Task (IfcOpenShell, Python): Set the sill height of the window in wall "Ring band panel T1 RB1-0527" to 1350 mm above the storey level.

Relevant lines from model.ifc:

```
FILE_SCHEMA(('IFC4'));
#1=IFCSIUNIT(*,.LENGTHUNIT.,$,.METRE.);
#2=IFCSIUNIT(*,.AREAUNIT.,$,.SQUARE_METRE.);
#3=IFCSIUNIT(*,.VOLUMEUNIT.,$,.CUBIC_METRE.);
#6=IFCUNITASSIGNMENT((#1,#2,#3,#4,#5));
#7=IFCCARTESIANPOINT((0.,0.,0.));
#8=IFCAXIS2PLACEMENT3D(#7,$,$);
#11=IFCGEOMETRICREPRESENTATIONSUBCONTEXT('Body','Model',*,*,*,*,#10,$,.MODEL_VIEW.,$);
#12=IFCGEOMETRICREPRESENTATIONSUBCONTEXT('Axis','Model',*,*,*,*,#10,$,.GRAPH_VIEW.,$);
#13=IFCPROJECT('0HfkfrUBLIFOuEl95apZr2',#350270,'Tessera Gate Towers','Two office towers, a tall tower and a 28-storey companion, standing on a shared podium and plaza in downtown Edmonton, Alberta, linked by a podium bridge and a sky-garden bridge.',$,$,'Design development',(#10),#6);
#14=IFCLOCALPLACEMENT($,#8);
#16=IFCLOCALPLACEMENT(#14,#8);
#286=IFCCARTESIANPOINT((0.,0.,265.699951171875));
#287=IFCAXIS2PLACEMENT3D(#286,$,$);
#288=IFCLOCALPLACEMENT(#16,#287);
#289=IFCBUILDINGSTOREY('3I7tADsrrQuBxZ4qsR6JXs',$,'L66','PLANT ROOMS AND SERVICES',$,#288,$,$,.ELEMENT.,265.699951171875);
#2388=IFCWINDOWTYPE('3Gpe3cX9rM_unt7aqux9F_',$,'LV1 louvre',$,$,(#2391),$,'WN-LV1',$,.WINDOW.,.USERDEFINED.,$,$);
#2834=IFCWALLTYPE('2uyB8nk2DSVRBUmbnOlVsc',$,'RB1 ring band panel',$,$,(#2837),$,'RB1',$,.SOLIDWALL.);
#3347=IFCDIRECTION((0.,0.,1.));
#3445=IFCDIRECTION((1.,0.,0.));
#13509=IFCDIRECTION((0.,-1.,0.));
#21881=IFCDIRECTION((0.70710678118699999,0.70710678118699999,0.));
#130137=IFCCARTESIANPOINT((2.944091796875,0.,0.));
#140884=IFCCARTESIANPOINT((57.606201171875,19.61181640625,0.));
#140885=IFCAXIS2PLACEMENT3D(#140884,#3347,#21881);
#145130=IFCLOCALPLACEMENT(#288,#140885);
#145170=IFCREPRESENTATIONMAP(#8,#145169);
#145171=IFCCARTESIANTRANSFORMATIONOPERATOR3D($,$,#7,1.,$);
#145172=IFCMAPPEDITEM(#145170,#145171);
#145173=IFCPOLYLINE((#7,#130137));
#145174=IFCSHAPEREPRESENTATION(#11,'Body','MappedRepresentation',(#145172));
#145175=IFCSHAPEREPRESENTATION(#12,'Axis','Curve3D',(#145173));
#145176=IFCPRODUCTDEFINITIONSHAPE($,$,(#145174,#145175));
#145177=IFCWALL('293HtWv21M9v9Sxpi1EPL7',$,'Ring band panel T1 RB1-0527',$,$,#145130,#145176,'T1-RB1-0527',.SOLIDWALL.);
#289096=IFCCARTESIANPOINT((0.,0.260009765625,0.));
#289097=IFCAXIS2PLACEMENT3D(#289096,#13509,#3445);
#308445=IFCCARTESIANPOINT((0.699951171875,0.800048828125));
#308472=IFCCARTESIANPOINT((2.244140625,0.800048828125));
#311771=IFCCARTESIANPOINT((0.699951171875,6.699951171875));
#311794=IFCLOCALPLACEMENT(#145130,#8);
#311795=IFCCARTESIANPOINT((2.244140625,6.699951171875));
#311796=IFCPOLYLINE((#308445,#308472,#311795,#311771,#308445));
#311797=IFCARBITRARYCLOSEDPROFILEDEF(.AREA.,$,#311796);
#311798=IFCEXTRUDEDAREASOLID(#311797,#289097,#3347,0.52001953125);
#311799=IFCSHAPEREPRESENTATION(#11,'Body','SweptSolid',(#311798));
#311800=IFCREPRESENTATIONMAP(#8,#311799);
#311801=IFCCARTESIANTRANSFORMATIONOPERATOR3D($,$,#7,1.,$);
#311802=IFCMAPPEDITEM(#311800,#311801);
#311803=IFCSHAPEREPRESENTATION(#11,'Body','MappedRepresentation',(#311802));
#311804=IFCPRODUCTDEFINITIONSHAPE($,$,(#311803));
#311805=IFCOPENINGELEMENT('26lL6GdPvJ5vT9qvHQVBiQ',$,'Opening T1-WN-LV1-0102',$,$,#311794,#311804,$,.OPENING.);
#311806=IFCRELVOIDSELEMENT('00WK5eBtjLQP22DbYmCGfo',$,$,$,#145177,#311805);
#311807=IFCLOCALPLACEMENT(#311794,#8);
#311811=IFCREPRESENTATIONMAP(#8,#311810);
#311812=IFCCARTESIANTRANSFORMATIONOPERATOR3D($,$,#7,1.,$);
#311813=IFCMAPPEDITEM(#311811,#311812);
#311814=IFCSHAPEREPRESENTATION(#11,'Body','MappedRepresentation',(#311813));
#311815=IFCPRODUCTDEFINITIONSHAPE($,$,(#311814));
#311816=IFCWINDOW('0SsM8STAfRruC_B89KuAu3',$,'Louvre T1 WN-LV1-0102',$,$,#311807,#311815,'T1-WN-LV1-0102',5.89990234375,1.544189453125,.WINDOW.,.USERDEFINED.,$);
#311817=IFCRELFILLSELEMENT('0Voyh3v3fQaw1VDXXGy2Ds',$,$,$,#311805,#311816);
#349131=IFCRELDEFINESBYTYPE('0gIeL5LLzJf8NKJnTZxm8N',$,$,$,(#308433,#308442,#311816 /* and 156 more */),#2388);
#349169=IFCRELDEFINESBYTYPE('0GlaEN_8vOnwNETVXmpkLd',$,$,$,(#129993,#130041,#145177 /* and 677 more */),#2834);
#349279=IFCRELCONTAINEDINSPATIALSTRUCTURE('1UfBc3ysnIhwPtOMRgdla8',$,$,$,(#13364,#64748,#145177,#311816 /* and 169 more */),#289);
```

```python
import numpy as np
import ifcopenshell
import ifcopenshell.api.geometry
import ifcopenshell.geom
import ifcopenshell.util.element
import ifcopenshell.util.placement
import ifcopenshell.util.shape
import ifcopenshell.util.unit

model = ifcopenshell.open("model.ifc")
unit_scale = ifcopenshell.util.unit.calculate_unit_scale(model)

window = model.by_id(311816)
opening = window.FillsVoids[0].RelatingOpeningElement
storey = ifcopenshell.util.element.get_container(window, ifc_class="IfcBuildingStorey")
level = ifcopenshell.util.placement.get_local_placement(storey.ObjectPlacement)[2, 3]

# The opening's origin need not be at the sill, so measure its lowest point.
shape = ifcopenshell.geom.create_shape(ifcopenshell.geom.settings(), opening)
bottom = ifcopenshell.util.shape.get_shape_bottom_elevation(shape, shape.geometry) / unit_scale
dz = level + 1.35 - bottom

shift = np.array([0.0, 0.0, dz])
# The window is placed relative to its opening, so it follows when the opening moves.
matrix = ifcopenshell.util.placement.get_local_placement(opening.ObjectPlacement)
matrix[:3, 3] += shift
ifcopenshell.api.geometry.edit_object_placement(
    model, product=opening, matrix=matrix, is_si=False, should_transform_children=True
)

print(f"moved by {dz * unit_scale:+.3f} m")

model.write("model-out.ifc")
```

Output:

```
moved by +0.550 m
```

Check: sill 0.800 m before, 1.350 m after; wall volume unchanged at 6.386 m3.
